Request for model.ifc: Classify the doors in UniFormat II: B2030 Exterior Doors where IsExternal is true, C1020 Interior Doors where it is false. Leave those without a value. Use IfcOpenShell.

First a look at what the model holds.

```python
import ifcopenshell
import ifcopenshell.util.element

model = ifcopenshell.open("model.ifc")
print(model.schema)
print("classifications:", [c.Name for c in model.by_type("IfcClassification")])
values = [ifcopenshell.util.element.get_pset(e, "Pset_DoorCommon", "IsExternal") for e in model.by_type("IfcDoor")]
for value in (True, False, None):
    print("IsExternal", value, values.count(value))
```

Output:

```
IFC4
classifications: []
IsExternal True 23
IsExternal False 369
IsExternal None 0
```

```python
import ifcopenshell
import ifcopenshell.api.classification
import ifcopenshell.util.element

model = ifcopenshell.open("model.ifc")

system = ifcopenshell.api.classification.add_classification(model, classification="UniFormat II")

doors = model.by_type("IfcDoor")
external = {e: ifcopenshell.util.element.get_pset(e, "Pset_DoorCommon", "IsExternal") for e in doors}
for flag, code, name in ((True, "B2030", "Exterior Doors"), (False, "C1020", "Interior Doors")):
    products = [e for e in doors if external[e] is flag]
    ifcopenshell.api.classification.add_reference(
        model, products=products, classification=system, identification=code, name=name
    )
    print(code, len(products))

model.write("model_edited.ifc")
```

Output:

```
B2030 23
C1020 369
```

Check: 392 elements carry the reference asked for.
